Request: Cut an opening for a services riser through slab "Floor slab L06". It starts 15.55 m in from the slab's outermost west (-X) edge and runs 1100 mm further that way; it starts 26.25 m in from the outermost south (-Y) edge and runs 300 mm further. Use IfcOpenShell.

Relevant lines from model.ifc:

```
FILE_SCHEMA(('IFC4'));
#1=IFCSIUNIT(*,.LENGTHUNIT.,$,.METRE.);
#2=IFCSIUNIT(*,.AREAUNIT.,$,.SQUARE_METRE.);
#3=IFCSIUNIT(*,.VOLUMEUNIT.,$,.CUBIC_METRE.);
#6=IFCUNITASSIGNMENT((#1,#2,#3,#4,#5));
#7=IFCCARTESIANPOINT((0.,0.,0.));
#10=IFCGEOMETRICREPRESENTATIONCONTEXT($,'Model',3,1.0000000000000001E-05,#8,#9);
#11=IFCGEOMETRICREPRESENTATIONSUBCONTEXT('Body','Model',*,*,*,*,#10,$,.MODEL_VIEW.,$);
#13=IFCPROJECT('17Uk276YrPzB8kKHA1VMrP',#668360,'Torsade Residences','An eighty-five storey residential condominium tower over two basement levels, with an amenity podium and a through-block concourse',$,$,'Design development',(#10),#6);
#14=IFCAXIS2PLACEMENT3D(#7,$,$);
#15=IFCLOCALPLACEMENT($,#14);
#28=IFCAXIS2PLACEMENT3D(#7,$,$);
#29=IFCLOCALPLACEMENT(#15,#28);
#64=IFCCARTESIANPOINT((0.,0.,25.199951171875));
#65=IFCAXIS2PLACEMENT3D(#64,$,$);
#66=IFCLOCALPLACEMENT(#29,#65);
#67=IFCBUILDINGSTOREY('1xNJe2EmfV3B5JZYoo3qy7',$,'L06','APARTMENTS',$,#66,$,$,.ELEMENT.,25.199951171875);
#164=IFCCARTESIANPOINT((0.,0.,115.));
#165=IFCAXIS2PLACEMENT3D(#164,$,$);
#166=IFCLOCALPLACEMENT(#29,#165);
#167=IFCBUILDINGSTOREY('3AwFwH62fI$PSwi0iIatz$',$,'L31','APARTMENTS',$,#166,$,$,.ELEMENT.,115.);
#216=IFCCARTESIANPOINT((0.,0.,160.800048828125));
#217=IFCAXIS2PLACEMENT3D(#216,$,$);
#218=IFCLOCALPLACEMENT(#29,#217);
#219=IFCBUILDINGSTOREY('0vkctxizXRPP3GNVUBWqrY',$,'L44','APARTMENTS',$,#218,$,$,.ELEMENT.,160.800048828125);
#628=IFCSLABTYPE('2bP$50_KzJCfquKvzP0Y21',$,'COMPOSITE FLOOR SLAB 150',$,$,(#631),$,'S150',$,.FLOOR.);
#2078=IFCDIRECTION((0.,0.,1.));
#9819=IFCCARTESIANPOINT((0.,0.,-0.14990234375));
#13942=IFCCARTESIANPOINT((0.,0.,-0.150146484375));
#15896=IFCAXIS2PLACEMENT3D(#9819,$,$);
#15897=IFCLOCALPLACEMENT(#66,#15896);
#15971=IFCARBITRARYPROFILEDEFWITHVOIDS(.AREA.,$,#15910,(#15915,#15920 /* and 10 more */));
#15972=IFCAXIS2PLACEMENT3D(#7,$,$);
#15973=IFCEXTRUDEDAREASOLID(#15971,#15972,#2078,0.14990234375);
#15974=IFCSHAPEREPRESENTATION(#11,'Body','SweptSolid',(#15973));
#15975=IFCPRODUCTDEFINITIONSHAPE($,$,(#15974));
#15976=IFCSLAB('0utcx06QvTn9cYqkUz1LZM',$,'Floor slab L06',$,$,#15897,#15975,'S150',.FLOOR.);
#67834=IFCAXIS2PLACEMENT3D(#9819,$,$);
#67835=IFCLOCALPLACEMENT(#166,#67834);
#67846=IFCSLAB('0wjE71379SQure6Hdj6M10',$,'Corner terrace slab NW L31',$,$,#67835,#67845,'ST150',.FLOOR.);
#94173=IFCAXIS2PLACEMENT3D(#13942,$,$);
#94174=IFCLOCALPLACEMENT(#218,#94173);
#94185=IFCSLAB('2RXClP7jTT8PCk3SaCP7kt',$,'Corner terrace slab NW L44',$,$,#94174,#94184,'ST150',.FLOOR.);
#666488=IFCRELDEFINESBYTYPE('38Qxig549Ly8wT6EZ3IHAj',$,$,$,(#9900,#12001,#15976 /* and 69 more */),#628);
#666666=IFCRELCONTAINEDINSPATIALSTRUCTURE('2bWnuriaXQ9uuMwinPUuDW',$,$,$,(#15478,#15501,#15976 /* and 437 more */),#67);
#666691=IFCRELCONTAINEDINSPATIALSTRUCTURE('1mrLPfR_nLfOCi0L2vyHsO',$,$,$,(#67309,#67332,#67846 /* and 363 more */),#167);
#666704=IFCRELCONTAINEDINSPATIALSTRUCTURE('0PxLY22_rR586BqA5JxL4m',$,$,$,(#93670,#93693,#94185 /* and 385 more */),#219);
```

```python
import numpy as np
import ifcopenshell
import ifcopenshell.api.feature
import ifcopenshell.api.geometry
import ifcopenshell.api.root
import ifcopenshell.geom
import ifcopenshell.util.placement
import ifcopenshell.util.representation
import ifcopenshell.util.shape
import ifcopenshell.util.unit

model = ifcopenshell.open("model.ifc")
unit_scale = ifcopenshell.util.unit.calculate_unit_scale(model)
settings = ifcopenshell.geom.settings()


def volume(element):
    """Net volume in cubic metres, openings subtracted."""
    shape = ifcopenshell.geom.create_shape(settings, element)
    return ifcopenshell.util.shape.get_volume(shape.geometry)


slab = model.by_id(15976)
before = volume(slab)

# Extent in the slab's own axes, in metres. The edges named are its -X and -Y sides.
slab_shape = ifcopenshell.geom.create_shape(settings, slab)
vertices = ifcopenshell.util.shape.get_vertices(slab_shape.geometry)
x_min, y_min, bottom = vertices.min(axis=0)
top = vertices[:, 2].max()

opening = ifcopenshell.api.root.create_entity(model, ifc_class="IfcOpeningElement", name="Services riser opening", predefined_type="OPENING")
context = ifcopenshell.util.representation.get_context(model, "Model", "Body", "MODEL_VIEW")
width, depth = 1.1, 0.3
outline = [(0.0, 0.0), (width, 0.0), (width, depth), (0.0, depth), (0.0, 0.0)]
# Overshoot both faces by 50 mm so the cut is clean.
shape = ifcopenshell.api.geometry.add_slab_representation(
    model, context=context, depth=top - bottom + 0.1, polyline=outline
)
ifcopenshell.api.geometry.assign_representation(model, product=opening, representation=shape)

matrix = ifcopenshell.util.placement.get_local_placement(slab.ObjectPlacement)
matrix[:, 3] = matrix @ np.append(np.array([x_min + 15.55, y_min + 26.25, bottom - 0.05]) / unit_scale, 1.0)
ifcopenshell.api.geometry.edit_object_placement(model, product=opening, matrix=matrix, is_si=False)
ifcopenshell.api.feature.add_feature(model, feature=opening, element=slab)

after = volume(slab)

print(f"slab volume {before:.3f} -> {after:.3f} m3")

model.write("model_edited.ifc")
```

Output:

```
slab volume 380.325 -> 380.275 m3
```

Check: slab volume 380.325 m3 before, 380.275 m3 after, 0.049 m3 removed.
